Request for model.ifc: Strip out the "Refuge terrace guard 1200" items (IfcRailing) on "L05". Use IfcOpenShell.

First a look at what the model holds.

```python
import ifcopenshell
import ifcopenshell.util.element

model = ifcopenshell.open("model.ifc")
print(model.schema)
storey = next(s for s in model.by_type("IfcBuildingStorey") if s.Name == "L05")
railings = [e for e in ifcopenshell.util.element.get_decomposition(storey) if e.is_a("IfcRailing")]
seen = {}
for e in railings:
    element_type = ifcopenshell.util.element.get_type(e)
    name = element_type.Name if element_type not in (None, e) else None
    seen[name] = seen.get(name, 0) + 1
for name, count in sorted(seen.items(), key=str):
    print(count, "x", name)
```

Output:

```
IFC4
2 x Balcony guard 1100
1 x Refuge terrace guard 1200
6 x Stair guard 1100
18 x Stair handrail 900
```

```python
import ifcopenshell
import ifcopenshell.api.root
import ifcopenshell.util.element

model = ifcopenshell.open("model.ifc")

storey = next(s for s in model.by_type("IfcBuildingStorey") if s.Name == "L05")
railings = [e for e in ifcopenshell.util.element.get_decomposition(storey) if e.is_a("IfcRailing")]
targets = [e for e in railings if (t := ifcopenshell.util.element.get_type(e)) not in (None, e) and t.Name == "Refuge terrace guard 1200"]

for e in targets:
    ifcopenshell.api.root.remove_product(model, product=e)
print(len(targets), "removed")

model.write("model_edited.ifc")
```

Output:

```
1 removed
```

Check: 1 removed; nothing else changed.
